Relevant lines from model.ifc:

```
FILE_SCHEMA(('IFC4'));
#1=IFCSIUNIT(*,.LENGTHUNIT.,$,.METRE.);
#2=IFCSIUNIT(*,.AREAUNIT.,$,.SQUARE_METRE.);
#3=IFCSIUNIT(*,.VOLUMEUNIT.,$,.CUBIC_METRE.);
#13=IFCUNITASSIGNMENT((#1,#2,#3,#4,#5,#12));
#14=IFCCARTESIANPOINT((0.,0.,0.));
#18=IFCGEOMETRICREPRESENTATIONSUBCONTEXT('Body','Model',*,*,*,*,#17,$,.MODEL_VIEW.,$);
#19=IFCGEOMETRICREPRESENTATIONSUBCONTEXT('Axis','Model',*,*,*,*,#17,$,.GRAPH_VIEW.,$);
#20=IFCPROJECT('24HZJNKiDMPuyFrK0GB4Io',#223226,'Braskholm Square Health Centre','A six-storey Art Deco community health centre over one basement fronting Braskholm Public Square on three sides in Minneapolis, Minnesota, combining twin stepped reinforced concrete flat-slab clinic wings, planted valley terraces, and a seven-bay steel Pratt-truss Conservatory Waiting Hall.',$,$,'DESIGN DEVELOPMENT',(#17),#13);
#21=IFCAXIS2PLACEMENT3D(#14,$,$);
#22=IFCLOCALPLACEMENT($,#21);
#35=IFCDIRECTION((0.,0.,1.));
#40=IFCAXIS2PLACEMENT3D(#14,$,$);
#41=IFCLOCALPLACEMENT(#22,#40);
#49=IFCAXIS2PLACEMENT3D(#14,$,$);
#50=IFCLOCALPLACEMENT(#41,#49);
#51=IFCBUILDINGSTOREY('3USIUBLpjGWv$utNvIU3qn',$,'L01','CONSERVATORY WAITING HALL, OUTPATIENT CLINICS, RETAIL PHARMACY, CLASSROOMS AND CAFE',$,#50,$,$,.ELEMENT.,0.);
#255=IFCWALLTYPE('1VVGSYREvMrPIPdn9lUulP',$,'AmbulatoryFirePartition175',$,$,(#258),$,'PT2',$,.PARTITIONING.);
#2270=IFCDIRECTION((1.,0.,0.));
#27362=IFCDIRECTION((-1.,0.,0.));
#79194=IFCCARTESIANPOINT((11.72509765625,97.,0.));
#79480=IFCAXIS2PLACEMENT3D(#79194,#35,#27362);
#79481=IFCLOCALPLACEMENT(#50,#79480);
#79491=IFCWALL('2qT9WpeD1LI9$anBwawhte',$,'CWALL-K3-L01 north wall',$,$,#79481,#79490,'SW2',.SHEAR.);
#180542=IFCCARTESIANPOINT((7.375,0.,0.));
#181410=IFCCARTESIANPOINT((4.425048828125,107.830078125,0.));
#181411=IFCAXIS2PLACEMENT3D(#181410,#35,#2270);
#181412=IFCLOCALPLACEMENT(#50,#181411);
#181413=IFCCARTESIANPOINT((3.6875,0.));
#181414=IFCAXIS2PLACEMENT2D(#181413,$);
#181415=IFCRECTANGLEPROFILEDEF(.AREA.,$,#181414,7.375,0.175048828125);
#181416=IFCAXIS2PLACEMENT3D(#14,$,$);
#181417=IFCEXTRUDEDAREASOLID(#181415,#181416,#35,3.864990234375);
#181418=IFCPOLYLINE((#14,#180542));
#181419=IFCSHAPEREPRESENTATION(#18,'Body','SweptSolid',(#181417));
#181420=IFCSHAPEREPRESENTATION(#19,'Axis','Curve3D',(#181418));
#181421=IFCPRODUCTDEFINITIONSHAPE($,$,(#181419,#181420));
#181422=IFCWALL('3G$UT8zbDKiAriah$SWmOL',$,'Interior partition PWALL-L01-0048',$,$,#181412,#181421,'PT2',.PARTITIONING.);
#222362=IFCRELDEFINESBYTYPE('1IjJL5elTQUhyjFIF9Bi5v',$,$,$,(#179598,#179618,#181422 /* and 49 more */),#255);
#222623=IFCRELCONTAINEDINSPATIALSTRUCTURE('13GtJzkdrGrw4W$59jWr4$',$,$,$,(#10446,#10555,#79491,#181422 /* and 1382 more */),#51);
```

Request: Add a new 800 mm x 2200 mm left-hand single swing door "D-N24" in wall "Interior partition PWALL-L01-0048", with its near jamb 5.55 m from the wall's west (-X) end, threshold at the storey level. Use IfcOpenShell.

```python
import numpy as np
import ifcopenshell
import ifcopenshell.api.feature
import ifcopenshell.api.geometry
import ifcopenshell.api.root
import ifcopenshell.api.spatial
import ifcopenshell.geom
import ifcopenshell.util.element
import ifcopenshell.util.placement
import ifcopenshell.util.representation
import ifcopenshell.util.shape
import ifcopenshell.util.unit

model = ifcopenshell.open("model.ifc")
unit_scale = ifcopenshell.util.unit.calculate_unit_scale(model)
settings = ifcopenshell.geom.settings()


def volume(element):
    """Net volume in cubic metres, openings subtracted."""
    shape = ifcopenshell.geom.create_shape(settings, element)
    return ifcopenshell.util.shape.get_volume(shape.geometry)


wall = model.by_id(181422)
storey = ifcopenshell.util.element.get_container(wall, ifc_class="IfcBuildingStorey")
context = ifcopenshell.util.representation.get_context(model, "Model", "Body", "MODEL_VIEW")
before = volume(wall)

width, height, from_end, sill = 0.8, 2.2, 5.55, 0.0  # metres

# The wall runs along its own X axis, and the end named is its -X end.
wall_shape = ifcopenshell.geom.create_shape(settings, wall)
x, y, z = ifcopenshell.util.shape.get_vertices(wall_shape.geometry).T
start = x.min() + from_end
face, thickness = float(y.min()), float(y.max() - y.min())
wall_matrix = ifcopenshell.util.placement.get_local_placement(wall.ObjectPlacement)
level = ifcopenshell.util.placement.get_local_placement(storey.ObjectPlacement)[2, 3]


def in_wall(x, y):
    """Placement at x, y metres in the wall's axes, at sill height."""
    matrix = wall_matrix.copy()
    matrix[:, 3] = wall_matrix @ np.array([x / unit_scale, y / unit_scale, 0.0, 1.0])
    matrix[2, 3] = level + sill / unit_scale
    return matrix


# Opening: a box that overshoots both wall faces by 50 mm.
opening = ifcopenshell.api.root.create_entity(model, ifc_class="IfcOpeningElement", predefined_type="OPENING")
box = ifcopenshell.api.geometry.add_wall_representation(
    model, context=context, length=width, height=height, thickness=thickness + 0.1
)
ifcopenshell.api.geometry.assign_representation(model, product=opening, representation=box)
ifcopenshell.api.geometry.edit_object_placement(model, product=opening, matrix=in_wall(start, face - 0.05), is_si=False)
ifcopenshell.api.feature.add_feature(model, feature=opening, element=wall)

door = ifcopenshell.api.root.create_entity(model, ifc_class="IfcDoor", name="D-N24", predefined_type="DOOR")
door.OverallWidth, door.OverallHeight = width / unit_scale, height / unit_scale
door.OperationType = "SINGLE_SWING_LEFT"
body = ifcopenshell.api.geometry.add_door_representation(
    model,
    context=context,
    overall_width=door.OverallWidth,
    overall_height=door.OverallHeight,
    operation_type="SINGLE_SWING_LEFT",
    lining_properties={"LiningDepth": thickness / unit_scale, "ThresholdDepth": thickness / unit_scale},
)
ifcopenshell.api.geometry.assign_representation(model, product=door, representation=body)
ifcopenshell.api.spatial.assign_container(model, products=[door], relating_structure=storey)
ifcopenshell.api.feature.add_filling(model, opening=opening, element=door)

# The lining spans the wall, so the door starts at the wall face.
ifcopenshell.api.geometry.edit_object_placement(model, product=door, matrix=in_wall(start, face), is_si=False)

after = volume(wall)

print(f"wall volume {before:.3f} -> {after:.3f} m3")

model.write("model-out.ifc")
```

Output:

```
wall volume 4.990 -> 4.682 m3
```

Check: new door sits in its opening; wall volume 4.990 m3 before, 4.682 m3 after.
